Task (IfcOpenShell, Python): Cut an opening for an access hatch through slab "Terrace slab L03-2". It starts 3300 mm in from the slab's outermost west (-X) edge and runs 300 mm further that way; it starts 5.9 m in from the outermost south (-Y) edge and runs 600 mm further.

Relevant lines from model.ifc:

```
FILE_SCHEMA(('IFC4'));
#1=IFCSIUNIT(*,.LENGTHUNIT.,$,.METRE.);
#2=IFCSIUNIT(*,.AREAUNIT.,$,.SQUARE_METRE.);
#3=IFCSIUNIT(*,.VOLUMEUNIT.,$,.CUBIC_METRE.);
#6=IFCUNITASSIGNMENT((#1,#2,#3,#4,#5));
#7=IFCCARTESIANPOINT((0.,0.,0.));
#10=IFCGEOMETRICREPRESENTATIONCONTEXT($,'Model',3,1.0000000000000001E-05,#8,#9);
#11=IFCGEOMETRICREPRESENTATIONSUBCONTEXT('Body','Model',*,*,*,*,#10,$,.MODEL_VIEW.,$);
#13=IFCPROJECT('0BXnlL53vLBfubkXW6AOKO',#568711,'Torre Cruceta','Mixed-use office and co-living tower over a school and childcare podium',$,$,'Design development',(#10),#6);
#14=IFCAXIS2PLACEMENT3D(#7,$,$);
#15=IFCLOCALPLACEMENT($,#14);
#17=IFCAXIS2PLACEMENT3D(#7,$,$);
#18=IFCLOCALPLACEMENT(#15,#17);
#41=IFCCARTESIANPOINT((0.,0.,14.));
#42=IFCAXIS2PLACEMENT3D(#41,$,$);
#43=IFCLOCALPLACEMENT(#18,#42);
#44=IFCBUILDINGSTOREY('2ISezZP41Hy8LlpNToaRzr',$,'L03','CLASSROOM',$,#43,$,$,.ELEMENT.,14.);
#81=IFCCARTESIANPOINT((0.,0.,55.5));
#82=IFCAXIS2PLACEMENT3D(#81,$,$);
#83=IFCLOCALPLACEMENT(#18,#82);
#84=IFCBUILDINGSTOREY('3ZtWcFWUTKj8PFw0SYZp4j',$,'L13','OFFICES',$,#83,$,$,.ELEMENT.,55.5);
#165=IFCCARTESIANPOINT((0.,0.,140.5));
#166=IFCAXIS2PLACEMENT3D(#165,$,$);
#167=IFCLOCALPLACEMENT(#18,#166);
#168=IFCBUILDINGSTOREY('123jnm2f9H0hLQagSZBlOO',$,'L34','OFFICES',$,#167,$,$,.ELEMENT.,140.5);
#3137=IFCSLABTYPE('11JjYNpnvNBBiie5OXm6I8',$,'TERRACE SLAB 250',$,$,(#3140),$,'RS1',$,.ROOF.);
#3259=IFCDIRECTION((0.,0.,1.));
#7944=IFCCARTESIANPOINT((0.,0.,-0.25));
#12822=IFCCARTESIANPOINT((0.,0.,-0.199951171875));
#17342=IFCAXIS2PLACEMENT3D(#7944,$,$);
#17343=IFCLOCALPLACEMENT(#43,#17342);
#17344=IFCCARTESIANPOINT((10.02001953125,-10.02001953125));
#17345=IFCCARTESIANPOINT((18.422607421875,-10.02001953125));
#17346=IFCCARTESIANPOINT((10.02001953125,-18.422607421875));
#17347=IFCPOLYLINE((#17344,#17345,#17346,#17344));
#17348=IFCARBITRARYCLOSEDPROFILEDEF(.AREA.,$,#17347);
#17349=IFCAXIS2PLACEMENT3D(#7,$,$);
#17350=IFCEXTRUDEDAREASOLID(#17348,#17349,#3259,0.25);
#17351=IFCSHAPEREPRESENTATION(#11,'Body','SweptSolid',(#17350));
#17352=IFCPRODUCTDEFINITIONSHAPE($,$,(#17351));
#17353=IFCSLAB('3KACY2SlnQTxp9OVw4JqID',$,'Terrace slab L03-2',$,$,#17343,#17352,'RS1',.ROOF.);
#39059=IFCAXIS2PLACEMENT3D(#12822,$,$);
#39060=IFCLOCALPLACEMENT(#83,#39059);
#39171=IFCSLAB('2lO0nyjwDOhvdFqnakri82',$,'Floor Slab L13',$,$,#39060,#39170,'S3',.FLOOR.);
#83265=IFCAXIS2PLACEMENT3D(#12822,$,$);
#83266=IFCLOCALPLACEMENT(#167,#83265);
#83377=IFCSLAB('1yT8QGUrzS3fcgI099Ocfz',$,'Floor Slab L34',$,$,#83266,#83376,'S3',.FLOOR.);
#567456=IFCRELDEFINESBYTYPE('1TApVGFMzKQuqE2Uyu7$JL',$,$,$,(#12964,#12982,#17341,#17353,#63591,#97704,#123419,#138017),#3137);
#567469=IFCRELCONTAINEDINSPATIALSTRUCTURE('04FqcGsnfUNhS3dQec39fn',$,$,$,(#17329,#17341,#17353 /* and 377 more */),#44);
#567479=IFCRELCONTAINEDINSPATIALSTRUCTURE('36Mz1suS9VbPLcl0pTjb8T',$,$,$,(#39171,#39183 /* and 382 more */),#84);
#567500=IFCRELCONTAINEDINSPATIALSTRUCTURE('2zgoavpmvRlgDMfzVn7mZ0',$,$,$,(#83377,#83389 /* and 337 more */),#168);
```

```python
import numpy as np
import ifcopenshell
import ifcopenshell.api.feature
import ifcopenshell.api.geometry
import ifcopenshell.api.root
import ifcopenshell.geom
import ifcopenshell.util.placement
import ifcopenshell.util.representation
import ifcopenshell.util.shape
import ifcopenshell.util.unit

model = ifcopenshell.open("model.ifc")
unit_scale = ifcopenshell.util.unit.calculate_unit_scale(model)
settings = ifcopenshell.geom.settings()


def volume(element):
    """Net volume in cubic metres, openings subtracted."""
    shape = ifcopenshell.geom.create_shape(settings, element)
    return ifcopenshell.util.shape.get_volume(shape.geometry)


slab = model.by_guid("3KACY2SlnQTxp9OVw4JqID")
before = volume(slab)

# Extent in the slab's own axes, in metres. The edges named are its -X and -Y sides.
slab_shape = ifcopenshell.geom.create_shape(settings, slab)
vertices = ifcopenshell.util.shape.get_vertices(slab_shape.geometry)
x_min, y_min, bottom = vertices.min(axis=0)
top = vertices[:, 2].max()

opening = ifcopenshell.api.root.create_entity(model, ifc_class="IfcOpeningElement", name="Access hatch opening", predefined_type="OPENING")
context = ifcopenshell.util.representation.get_context(model, "Model", "Body", "MODEL_VIEW")
width, depth = 0.3, 0.6
outline = [(0.0, 0.0), (width, 0.0), (width, depth), (0.0, depth), (0.0, 0.0)]
# Overshoot both faces by 50 mm so the cut is clean.
shape = ifcopenshell.api.geometry.add_slab_representation(
    model, context=context, depth=top - bottom + 0.1, polyline=outline
)
ifcopenshell.api.geometry.assign_representation(model, product=opening, representation=shape)

matrix = ifcopenshell.util.placement.get_local_placement(slab.ObjectPlacement)
matrix[:, 3] = matrix @ np.append(np.array([x_min + 3.3, y_min + 5.9, bottom - 0.05]) / unit_scale, 1.0)
ifcopenshell.api.geometry.edit_object_placement(model, product=opening, matrix=matrix, is_si=False)
ifcopenshell.api.feature.add_feature(model, feature=opening, element=slab)

after = volume(slab)

print(f"slab volume {before:.3f} -> {after:.3f} m3")

model.write("model_updated.ifc")
```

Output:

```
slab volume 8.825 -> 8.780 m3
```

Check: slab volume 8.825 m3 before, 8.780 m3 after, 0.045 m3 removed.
